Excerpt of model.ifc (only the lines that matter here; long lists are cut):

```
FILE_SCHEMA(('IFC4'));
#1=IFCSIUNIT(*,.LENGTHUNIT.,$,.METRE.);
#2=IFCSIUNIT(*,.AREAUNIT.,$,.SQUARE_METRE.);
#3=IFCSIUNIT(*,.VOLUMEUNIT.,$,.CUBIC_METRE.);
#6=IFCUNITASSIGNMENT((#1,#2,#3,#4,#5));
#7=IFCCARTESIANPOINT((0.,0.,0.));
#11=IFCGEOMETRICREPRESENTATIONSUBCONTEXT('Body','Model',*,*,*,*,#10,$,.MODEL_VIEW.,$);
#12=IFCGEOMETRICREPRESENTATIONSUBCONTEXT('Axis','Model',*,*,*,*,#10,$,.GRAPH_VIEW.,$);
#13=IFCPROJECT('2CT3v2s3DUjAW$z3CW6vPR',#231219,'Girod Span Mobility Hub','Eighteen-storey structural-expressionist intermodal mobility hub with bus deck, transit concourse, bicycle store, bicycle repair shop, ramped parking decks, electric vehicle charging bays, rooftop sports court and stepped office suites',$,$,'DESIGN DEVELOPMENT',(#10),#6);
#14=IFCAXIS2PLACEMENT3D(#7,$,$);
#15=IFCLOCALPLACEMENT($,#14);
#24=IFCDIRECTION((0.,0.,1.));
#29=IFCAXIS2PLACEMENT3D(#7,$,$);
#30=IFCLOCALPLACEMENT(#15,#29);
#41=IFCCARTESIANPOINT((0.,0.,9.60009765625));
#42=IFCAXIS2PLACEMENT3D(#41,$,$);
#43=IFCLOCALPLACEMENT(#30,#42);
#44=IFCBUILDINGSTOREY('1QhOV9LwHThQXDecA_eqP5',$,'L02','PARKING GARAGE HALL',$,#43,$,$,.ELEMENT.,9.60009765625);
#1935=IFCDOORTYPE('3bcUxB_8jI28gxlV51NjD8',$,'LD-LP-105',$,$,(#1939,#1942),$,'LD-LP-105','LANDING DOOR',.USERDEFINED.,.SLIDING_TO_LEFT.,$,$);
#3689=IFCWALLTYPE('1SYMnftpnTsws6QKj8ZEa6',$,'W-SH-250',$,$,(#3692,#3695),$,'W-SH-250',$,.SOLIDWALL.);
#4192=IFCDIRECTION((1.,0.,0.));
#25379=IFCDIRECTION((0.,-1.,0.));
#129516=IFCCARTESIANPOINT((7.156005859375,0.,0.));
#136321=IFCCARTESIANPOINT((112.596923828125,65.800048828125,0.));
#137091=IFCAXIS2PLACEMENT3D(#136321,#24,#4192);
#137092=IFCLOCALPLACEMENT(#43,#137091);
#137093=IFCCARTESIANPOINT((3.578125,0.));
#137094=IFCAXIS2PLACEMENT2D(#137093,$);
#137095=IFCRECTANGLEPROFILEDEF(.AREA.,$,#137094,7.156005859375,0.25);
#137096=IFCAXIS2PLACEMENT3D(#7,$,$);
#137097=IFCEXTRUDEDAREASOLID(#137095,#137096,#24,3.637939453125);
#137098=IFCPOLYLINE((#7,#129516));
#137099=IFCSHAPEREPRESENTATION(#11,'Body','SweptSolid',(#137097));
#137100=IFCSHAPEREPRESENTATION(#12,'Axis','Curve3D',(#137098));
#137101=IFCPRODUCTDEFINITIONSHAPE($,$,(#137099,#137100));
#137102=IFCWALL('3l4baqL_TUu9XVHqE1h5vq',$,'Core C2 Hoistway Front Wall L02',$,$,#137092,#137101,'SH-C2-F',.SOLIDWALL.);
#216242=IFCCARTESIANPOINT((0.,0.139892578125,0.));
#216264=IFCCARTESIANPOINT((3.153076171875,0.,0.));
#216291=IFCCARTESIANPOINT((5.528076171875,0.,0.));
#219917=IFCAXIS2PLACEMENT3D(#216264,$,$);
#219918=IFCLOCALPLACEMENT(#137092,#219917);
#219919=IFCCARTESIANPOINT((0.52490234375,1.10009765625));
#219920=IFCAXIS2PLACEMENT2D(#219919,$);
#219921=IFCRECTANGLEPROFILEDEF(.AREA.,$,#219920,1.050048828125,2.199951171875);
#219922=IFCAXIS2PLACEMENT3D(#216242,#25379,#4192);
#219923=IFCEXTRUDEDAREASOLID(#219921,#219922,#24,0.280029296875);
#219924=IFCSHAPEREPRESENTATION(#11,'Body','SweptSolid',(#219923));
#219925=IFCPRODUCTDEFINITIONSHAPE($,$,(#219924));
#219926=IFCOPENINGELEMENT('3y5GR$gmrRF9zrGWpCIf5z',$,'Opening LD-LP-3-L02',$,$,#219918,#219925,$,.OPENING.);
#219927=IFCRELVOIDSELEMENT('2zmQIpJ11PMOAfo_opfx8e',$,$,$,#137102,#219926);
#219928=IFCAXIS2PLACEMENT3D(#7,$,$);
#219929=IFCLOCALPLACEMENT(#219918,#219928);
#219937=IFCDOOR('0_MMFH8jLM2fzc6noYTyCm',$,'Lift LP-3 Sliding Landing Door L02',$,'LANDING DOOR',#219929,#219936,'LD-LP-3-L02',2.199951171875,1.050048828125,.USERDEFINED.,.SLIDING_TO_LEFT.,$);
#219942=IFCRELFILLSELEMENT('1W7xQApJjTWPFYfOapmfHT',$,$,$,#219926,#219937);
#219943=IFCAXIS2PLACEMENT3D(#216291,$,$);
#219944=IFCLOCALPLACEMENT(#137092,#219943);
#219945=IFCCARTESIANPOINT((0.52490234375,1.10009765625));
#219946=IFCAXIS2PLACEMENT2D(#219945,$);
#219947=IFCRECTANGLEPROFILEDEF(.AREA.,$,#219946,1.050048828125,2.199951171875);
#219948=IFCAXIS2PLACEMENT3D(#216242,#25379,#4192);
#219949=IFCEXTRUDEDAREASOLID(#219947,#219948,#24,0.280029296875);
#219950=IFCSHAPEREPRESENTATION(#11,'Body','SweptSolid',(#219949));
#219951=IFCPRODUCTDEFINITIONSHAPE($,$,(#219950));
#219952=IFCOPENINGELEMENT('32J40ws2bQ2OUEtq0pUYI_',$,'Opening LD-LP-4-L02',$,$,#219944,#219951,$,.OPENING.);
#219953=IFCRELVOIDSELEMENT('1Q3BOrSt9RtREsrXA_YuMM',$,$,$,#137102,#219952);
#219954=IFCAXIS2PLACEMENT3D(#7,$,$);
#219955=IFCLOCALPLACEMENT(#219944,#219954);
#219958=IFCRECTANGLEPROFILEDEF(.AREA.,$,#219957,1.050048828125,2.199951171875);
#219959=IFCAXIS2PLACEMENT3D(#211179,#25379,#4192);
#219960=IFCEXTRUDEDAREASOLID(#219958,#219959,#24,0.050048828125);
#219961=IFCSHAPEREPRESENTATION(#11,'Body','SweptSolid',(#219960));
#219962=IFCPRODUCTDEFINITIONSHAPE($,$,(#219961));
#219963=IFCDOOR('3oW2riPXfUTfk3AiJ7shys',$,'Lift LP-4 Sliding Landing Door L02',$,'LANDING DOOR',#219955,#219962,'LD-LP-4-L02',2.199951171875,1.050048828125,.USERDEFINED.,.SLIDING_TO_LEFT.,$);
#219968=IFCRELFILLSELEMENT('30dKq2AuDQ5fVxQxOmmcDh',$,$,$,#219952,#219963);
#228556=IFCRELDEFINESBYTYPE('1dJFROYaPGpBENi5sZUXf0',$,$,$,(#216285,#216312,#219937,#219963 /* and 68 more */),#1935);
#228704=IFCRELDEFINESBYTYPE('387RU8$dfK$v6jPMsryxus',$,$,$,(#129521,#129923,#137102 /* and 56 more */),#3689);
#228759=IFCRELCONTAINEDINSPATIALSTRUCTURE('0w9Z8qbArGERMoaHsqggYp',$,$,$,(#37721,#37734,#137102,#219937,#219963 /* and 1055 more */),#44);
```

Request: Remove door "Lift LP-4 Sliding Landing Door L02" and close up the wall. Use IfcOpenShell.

```python
import ifcopenshell
import ifcopenshell.api.feature
import ifcopenshell.api.root
import ifcopenshell.geom
import ifcopenshell.util.shape

model = ifcopenshell.open("model.ifc")
settings = ifcopenshell.geom.settings()


def volume(element):
    """Net volume in cubic metres, openings subtracted."""
    shape = ifcopenshell.geom.create_shape(settings, element)
    return ifcopenshell.util.shape.get_volume(shape.geometry)


door = model.by_guid("3oW2riPXfUTfk3AiJ7shys")
opening = door.FillsVoids[0].RelatingOpeningElement
wall = opening.VoidsElements[0].RelatingBuildingElement
before = volume(wall)

ifcopenshell.api.root.remove_product(model, product=door)
ifcopenshell.api.feature.remove_feature(model, feature=opening)

after = volume(wall)

print(f"wall volume {before:.3f} -> {after:.3f} m3")

model.write("model_edited.ifc")
```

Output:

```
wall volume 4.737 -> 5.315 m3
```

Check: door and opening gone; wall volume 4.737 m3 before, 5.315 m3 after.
